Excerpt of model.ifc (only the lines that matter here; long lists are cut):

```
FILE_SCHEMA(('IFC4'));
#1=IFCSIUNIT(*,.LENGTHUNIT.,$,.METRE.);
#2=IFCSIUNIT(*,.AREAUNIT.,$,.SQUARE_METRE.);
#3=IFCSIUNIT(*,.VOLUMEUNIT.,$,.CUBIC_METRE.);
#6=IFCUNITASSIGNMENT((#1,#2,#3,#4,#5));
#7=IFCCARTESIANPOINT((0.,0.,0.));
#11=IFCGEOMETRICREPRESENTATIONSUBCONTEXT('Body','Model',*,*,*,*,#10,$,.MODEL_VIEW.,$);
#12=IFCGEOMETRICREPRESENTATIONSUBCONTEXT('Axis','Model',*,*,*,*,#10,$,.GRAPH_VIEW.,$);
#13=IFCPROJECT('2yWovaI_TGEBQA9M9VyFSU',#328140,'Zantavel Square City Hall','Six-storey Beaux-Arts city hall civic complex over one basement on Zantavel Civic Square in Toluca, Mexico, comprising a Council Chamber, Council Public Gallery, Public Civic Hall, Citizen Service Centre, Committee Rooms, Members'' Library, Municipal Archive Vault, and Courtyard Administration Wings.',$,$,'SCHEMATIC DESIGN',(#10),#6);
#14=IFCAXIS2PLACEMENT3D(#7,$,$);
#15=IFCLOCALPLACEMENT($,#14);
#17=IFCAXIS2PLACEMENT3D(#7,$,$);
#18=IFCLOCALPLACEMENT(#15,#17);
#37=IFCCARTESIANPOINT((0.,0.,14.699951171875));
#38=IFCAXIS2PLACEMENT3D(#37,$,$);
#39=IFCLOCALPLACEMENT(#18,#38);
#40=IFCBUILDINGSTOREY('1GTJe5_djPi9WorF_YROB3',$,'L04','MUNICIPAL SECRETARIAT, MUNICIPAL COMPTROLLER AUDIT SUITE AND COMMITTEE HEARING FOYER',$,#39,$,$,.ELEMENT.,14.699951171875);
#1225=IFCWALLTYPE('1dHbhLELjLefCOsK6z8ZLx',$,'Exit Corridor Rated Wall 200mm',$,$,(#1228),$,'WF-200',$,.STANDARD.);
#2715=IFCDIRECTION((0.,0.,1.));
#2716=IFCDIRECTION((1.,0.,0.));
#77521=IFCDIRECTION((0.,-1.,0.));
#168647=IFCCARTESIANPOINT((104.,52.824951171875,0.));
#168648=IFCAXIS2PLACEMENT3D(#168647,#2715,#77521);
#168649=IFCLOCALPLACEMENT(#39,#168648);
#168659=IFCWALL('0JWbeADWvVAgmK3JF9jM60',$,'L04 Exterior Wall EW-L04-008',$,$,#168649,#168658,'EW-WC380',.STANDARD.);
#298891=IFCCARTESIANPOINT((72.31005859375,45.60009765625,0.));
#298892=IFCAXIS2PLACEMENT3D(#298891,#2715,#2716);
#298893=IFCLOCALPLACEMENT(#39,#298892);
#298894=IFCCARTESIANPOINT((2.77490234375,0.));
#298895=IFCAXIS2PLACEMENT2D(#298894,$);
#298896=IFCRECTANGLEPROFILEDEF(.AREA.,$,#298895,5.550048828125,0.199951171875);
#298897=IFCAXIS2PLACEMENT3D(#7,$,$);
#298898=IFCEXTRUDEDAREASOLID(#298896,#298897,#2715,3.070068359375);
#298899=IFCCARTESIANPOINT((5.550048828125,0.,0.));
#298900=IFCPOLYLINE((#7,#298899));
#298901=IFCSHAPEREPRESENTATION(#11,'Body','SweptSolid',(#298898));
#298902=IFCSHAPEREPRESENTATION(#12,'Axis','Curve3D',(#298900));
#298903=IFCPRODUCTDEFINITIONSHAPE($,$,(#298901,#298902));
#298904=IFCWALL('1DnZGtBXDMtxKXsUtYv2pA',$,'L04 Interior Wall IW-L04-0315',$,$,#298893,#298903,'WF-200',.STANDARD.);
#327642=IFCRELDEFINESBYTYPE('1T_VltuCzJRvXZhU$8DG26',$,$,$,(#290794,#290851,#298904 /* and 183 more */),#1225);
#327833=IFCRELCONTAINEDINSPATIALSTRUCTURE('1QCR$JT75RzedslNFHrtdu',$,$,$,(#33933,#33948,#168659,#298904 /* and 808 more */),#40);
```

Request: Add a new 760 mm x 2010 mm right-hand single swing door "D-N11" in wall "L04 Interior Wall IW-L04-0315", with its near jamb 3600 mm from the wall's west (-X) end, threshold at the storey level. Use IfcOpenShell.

```python
import numpy as np
import ifcopenshell
import ifcopenshell.api.feature
import ifcopenshell.api.geometry
import ifcopenshell.api.root
import ifcopenshell.api.spatial
import ifcopenshell.geom
import ifcopenshell.util.element
import ifcopenshell.util.placement
import ifcopenshell.util.representation
import ifcopenshell.util.shape
import ifcopenshell.util.unit

model = ifcopenshell.open("model.ifc")
unit_scale = ifcopenshell.util.unit.calculate_unit_scale(model)
settings = ifcopenshell.geom.settings()


def volume(element):
    """Net volume in cubic metres, openings subtracted."""
    shape = ifcopenshell.geom.create_shape(settings, element)
    return ifcopenshell.util.shape.get_volume(shape.geometry)


wall = model.by_guid("1DnZGtBXDMtxKXsUtYv2pA")
storey = ifcopenshell.util.element.get_container(wall, ifc_class="IfcBuildingStorey")
context = ifcopenshell.util.representation.get_context(model, "Model", "Body", "MODEL_VIEW")
before = volume(wall)

width, height, from_end, sill = 0.76, 2.01, 3.6, 0.0  # metres

# The wall runs along its own X axis, and the end named is its -X end.
wall_shape = ifcopenshell.geom.create_shape(settings, wall)
x, y, z = ifcopenshell.util.shape.get_vertices(wall_shape.geometry).T
start = x.min() + from_end
face, thickness = float(y.min()), float(y.max() - y.min())
wall_matrix = ifcopenshell.util.placement.get_local_placement(wall.ObjectPlacement)
level = ifcopenshell.util.placement.get_local_placement(storey.ObjectPlacement)[2, 3]


def in_wall(x, y):
    """Placement at x, y metres in the wall's axes, at sill height."""
    matrix = wall_matrix.copy()
    matrix[:, 3] = wall_matrix @ np.array([x / unit_scale, y / unit_scale, 0.0, 1.0])
    matrix[2, 3] = level + sill / unit_scale
    return matrix


# Opening: a box that overshoots both wall faces by 50 mm.
opening = ifcopenshell.api.root.create_entity(model, ifc_class="IfcOpeningElement", predefined_type="OPENING")
box = ifcopenshell.api.geometry.add_wall_representation(
    model, context=context, length=width, height=height, thickness=thickness + 0.1
)
ifcopenshell.api.geometry.assign_representation(model, product=opening, representation=box)
ifcopenshell.api.geometry.edit_object_placement(model, product=opening, matrix=in_wall(start, face - 0.05), is_si=False)
ifcopenshell.api.feature.add_feature(model, feature=opening, element=wall)

door = ifcopenshell.api.root.create_entity(model, ifc_class="IfcDoor", name="D-N11", predefined_type="DOOR")
door.OverallWidth, door.OverallHeight = width / unit_scale, height / unit_scale
door.OperationType = "SINGLE_SWING_RIGHT"
body = ifcopenshell.api.geometry.add_door_representation(
    model,
    context=context,
    overall_width=door.OverallWidth,
    overall_height=door.OverallHeight,
    operation_type="SINGLE_SWING_RIGHT",
    lining_properties={"LiningDepth": thickness / unit_scale, "ThresholdDepth": thickness / unit_scale},
)
ifcopenshell.api.geometry.assign_representation(model, product=door, representation=body)
ifcopenshell.api.spatial.assign_container(model, products=[door], relating_structure=storey)
ifcopenshell.api.feature.add_filling(model, opening=opening, element=door)

# The lining spans the wall, so the door starts at the wall face.
ifcopenshell.api.geometry.edit_object_placement(model, product=door, matrix=in_wall(start, face), is_si=False)

after = volume(wall)

print(f"wall volume {before:.3f} -> {after:.3f} m3")

model.write("model-out.ifc")
```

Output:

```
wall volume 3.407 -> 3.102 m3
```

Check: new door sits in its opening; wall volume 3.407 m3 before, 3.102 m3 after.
